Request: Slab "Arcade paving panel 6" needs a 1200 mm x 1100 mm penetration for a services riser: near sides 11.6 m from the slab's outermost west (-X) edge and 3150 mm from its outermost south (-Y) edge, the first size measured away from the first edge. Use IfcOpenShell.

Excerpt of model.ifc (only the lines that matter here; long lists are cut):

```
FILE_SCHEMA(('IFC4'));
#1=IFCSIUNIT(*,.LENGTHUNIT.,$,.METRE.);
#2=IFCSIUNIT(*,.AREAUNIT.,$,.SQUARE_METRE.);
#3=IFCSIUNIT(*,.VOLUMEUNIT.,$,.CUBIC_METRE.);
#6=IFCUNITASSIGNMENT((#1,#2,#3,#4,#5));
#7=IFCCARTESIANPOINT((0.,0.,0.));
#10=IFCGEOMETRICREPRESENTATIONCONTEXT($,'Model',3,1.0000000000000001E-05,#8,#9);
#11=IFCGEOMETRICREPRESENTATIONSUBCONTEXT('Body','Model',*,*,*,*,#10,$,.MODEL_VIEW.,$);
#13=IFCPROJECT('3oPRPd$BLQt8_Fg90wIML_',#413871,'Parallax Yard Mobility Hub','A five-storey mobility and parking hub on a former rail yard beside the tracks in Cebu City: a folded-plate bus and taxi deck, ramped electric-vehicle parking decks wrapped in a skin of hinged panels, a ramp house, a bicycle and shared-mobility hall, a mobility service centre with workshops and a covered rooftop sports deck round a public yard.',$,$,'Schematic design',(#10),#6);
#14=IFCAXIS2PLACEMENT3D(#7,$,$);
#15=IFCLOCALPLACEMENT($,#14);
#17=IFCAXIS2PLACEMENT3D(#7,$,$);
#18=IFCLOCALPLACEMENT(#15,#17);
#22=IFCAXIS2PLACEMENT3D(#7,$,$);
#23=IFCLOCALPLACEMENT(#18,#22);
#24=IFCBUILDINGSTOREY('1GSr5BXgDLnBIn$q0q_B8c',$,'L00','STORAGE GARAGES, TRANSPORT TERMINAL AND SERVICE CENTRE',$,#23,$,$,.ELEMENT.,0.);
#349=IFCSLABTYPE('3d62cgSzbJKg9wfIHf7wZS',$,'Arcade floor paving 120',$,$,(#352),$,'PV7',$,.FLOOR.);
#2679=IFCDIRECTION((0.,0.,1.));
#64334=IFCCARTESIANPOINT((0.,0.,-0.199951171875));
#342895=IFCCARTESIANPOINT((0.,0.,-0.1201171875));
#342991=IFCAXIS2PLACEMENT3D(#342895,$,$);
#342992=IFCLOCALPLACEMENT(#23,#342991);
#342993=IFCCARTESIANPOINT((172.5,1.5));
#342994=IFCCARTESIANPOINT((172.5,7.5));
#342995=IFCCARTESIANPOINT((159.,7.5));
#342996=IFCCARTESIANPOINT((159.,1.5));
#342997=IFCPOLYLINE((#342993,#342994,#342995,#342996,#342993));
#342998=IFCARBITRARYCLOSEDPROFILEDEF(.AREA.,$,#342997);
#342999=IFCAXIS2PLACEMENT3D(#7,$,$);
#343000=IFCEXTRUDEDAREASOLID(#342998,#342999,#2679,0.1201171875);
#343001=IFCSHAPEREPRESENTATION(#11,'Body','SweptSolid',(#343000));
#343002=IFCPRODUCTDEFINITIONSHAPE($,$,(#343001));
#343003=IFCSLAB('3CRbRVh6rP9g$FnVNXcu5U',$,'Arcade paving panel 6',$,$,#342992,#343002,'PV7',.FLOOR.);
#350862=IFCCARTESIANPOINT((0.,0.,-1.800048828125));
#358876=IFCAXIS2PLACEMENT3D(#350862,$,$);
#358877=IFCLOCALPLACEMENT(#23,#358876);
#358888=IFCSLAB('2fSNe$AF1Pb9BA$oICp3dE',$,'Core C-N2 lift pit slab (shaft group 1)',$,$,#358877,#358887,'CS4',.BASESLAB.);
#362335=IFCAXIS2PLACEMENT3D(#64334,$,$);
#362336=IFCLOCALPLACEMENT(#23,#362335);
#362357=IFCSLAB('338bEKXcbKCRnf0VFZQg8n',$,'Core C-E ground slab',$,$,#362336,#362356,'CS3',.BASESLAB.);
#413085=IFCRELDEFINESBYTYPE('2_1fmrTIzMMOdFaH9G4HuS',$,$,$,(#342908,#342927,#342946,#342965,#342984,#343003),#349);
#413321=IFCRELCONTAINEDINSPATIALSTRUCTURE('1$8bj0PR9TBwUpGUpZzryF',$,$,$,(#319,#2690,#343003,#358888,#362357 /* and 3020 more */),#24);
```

```python
import numpy as np
import ifcopenshell
import ifcopenshell.api.feature
import ifcopenshell.api.geometry
import ifcopenshell.api.root
import ifcopenshell.geom
import ifcopenshell.util.placement
import ifcopenshell.util.representation
import ifcopenshell.util.shape
import ifcopenshell.util.unit

model = ifcopenshell.open("model.ifc")
unit_scale = ifcopenshell.util.unit.calculate_unit_scale(model)
settings = ifcopenshell.geom.settings()


def volume(element):
    """Net volume in cubic metres, openings subtracted."""
    shape = ifcopenshell.geom.create_shape(settings, element)
    return ifcopenshell.util.shape.get_volume(shape.geometry)


slab = model.by_id(343003)
before = volume(slab)

# Extent in the slab's own axes, in metres. The edges named are its -X and -Y sides.
slab_shape = ifcopenshell.geom.create_shape(settings, slab)
vertices = ifcopenshell.util.shape.get_vertices(slab_shape.geometry)
x_min, y_min, bottom = vertices.min(axis=0)
top = vertices[:, 2].max()

opening = ifcopenshell.api.root.create_entity(model, ifc_class="IfcOpeningElement", name="Services riser opening", predefined_type="OPENING")
context = ifcopenshell.util.representation.get_context(model, "Model", "Body", "MODEL_VIEW")
width, depth = 1.2, 1.1
outline = [(0.0, 0.0), (width, 0.0), (width, depth), (0.0, depth), (0.0, 0.0)]
# Overshoot both faces by 50 mm so the cut is clean.
shape = ifcopenshell.api.geometry.add_slab_representation(
    model, context=context, depth=top - bottom + 0.1, polyline=outline
)
ifcopenshell.api.geometry.assign_representation(model, product=opening, representation=shape)

matrix = ifcopenshell.util.placement.get_local_placement(slab.ObjectPlacement)
matrix[:, 3] = matrix @ np.append(np.array([x_min + 11.6, y_min + 3.15, bottom - 0.05]) / unit_scale, 1.0)
ifcopenshell.api.geometry.edit_object_placement(model, product=opening, matrix=matrix, is_si=False)
ifcopenshell.api.feature.add_feature(model, feature=opening, element=slab)

after = volume(slab)

print(f"slab volume {before:.3f} -> {after:.3f} m3")

model.write("model_updated.ifc")
```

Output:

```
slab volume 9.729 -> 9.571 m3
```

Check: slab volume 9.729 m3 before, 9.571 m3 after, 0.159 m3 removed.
